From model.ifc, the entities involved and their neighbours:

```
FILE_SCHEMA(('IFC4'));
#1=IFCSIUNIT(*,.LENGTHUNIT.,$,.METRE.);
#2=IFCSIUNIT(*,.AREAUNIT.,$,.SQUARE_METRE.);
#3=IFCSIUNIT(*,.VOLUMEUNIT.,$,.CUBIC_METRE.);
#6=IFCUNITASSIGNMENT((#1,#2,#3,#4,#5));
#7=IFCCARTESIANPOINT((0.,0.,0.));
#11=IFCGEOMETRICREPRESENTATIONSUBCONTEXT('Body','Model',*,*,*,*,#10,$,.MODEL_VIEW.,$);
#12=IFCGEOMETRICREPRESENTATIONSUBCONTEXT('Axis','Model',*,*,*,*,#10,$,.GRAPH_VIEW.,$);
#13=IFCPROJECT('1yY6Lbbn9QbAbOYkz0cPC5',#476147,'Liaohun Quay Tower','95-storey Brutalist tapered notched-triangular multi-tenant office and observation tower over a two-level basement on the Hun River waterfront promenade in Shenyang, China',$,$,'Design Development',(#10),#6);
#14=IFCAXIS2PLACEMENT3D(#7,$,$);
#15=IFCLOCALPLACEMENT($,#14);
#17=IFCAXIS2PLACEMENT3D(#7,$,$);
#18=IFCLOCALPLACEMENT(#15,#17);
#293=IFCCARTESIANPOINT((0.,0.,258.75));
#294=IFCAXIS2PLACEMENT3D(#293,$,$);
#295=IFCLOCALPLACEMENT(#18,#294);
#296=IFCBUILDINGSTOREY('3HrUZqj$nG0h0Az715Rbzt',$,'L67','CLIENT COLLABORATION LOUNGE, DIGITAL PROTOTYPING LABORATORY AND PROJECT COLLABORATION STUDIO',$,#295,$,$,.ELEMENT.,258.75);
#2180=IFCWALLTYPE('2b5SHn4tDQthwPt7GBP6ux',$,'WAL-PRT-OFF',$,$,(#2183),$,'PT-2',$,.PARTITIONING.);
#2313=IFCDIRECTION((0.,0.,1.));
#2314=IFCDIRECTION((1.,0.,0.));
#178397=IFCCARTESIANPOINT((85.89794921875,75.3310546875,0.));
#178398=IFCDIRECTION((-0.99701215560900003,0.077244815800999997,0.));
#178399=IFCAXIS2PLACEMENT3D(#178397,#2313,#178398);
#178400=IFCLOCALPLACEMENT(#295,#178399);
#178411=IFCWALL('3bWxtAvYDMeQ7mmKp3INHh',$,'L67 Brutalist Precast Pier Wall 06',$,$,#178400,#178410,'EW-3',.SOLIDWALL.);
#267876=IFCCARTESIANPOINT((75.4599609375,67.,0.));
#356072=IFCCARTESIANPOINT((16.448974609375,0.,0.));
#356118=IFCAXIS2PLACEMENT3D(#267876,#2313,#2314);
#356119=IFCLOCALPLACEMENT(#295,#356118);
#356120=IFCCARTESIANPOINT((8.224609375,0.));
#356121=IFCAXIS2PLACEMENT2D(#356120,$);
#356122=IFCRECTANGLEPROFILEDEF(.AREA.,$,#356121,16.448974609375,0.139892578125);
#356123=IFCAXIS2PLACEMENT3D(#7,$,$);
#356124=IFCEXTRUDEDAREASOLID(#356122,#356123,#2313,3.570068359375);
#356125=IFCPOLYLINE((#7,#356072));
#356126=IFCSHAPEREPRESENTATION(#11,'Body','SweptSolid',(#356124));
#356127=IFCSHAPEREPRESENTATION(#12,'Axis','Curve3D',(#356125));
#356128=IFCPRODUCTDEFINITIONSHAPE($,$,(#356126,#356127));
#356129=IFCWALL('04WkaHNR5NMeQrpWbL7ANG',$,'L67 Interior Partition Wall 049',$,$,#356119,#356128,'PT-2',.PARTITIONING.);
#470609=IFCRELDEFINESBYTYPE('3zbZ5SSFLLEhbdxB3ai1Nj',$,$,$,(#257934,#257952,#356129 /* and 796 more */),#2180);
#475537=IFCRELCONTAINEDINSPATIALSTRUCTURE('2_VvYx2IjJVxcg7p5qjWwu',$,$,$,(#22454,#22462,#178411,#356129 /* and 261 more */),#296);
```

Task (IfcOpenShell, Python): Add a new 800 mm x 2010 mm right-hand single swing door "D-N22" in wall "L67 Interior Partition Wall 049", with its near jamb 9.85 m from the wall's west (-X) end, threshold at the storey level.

```python
import numpy as np
import ifcopenshell
import ifcopenshell.api.feature
import ifcopenshell.api.geometry
import ifcopenshell.api.root
import ifcopenshell.api.spatial
import ifcopenshell.geom
import ifcopenshell.util.element
import ifcopenshell.util.placement
import ifcopenshell.util.representation
import ifcopenshell.util.shape
import ifcopenshell.util.unit

model = ifcopenshell.open("model.ifc")
unit_scale = ifcopenshell.util.unit.calculate_unit_scale(model)
settings = ifcopenshell.geom.settings()


def volume(element):
    """Net volume in cubic metres, openings subtracted."""
    shape = ifcopenshell.geom.create_shape(settings, element)
    return ifcopenshell.util.shape.get_volume(shape.geometry)


wall = model.by_guid("04WkaHNR5NMeQrpWbL7ANG")
storey = ifcopenshell.util.element.get_container(wall, ifc_class="IfcBuildingStorey")
context = ifcopenshell.util.representation.get_context(model, "Model", "Body", "MODEL_VIEW")
before = volume(wall)

width, height, from_end, sill = 0.8, 2.01, 9.85, 0.0  # metres

# The wall runs along its own X axis, and the end named is its -X end.
wall_shape = ifcopenshell.geom.create_shape(settings, wall)
x, y, z = ifcopenshell.util.shape.get_vertices(wall_shape.geometry).T
start = x.min() + from_end
face, thickness = float(y.min()), float(y.max() - y.min())
wall_matrix = ifcopenshell.util.placement.get_local_placement(wall.ObjectPlacement)
level = ifcopenshell.util.placement.get_local_placement(storey.ObjectPlacement)[2, 3]


def in_wall(x, y):
    """Placement at x, y metres in the wall's axes, at sill height."""
    matrix = wall_matrix.copy()
    matrix[:, 3] = wall_matrix @ np.array([x / unit_scale, y / unit_scale, 0.0, 1.0])
    matrix[2, 3] = level + sill / unit_scale
    return matrix


# Opening: a box that overshoots both wall faces by 50 mm.
opening = ifcopenshell.api.root.create_entity(model, ifc_class="IfcOpeningElement", predefined_type="OPENING")
box = ifcopenshell.api.geometry.add_wall_representation(
    model, context=context, length=width, height=height, thickness=thickness + 0.1
)
ifcopenshell.api.geometry.assign_representation(model, product=opening, representation=box)
ifcopenshell.api.geometry.edit_object_placement(model, product=opening, matrix=in_wall(start, face - 0.05), is_si=False)
ifcopenshell.api.feature.add_feature(model, feature=opening, element=wall)

door = ifcopenshell.api.root.create_entity(model, ifc_class="IfcDoor", name="D-N22", predefined_type="DOOR")
door.OverallWidth, door.OverallHeight = width / unit_scale, height / unit_scale
door.OperationType = "SINGLE_SWING_RIGHT"
body = ifcopenshell.api.geometry.add_door_representation(
    model,
    context=context,
    overall_width=door.OverallWidth,
    overall_height=door.OverallHeight,
    operation_type="SINGLE_SWING_RIGHT",
    lining_properties={"LiningDepth": thickness / unit_scale, "ThresholdDepth": thickness / unit_scale},
)
ifcopenshell.api.geometry.assign_representation(model, product=door, representation=body)
ifcopenshell.api.spatial.assign_container(model, products=[door], relating_structure=storey)
ifcopenshell.api.feature.add_filling(model, opening=opening, element=door)

# The lining spans the wall, so the door starts at the wall face.
ifcopenshell.api.geometry.edit_object_placement(model, product=door, matrix=in_wall(start, face), is_si=False)

after = volume(wall)

print(f"wall volume {before:.3f} -> {after:.3f} m3")

model.write("model_updated.ifc")
```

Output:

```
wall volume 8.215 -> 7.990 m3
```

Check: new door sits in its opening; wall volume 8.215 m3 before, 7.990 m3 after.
